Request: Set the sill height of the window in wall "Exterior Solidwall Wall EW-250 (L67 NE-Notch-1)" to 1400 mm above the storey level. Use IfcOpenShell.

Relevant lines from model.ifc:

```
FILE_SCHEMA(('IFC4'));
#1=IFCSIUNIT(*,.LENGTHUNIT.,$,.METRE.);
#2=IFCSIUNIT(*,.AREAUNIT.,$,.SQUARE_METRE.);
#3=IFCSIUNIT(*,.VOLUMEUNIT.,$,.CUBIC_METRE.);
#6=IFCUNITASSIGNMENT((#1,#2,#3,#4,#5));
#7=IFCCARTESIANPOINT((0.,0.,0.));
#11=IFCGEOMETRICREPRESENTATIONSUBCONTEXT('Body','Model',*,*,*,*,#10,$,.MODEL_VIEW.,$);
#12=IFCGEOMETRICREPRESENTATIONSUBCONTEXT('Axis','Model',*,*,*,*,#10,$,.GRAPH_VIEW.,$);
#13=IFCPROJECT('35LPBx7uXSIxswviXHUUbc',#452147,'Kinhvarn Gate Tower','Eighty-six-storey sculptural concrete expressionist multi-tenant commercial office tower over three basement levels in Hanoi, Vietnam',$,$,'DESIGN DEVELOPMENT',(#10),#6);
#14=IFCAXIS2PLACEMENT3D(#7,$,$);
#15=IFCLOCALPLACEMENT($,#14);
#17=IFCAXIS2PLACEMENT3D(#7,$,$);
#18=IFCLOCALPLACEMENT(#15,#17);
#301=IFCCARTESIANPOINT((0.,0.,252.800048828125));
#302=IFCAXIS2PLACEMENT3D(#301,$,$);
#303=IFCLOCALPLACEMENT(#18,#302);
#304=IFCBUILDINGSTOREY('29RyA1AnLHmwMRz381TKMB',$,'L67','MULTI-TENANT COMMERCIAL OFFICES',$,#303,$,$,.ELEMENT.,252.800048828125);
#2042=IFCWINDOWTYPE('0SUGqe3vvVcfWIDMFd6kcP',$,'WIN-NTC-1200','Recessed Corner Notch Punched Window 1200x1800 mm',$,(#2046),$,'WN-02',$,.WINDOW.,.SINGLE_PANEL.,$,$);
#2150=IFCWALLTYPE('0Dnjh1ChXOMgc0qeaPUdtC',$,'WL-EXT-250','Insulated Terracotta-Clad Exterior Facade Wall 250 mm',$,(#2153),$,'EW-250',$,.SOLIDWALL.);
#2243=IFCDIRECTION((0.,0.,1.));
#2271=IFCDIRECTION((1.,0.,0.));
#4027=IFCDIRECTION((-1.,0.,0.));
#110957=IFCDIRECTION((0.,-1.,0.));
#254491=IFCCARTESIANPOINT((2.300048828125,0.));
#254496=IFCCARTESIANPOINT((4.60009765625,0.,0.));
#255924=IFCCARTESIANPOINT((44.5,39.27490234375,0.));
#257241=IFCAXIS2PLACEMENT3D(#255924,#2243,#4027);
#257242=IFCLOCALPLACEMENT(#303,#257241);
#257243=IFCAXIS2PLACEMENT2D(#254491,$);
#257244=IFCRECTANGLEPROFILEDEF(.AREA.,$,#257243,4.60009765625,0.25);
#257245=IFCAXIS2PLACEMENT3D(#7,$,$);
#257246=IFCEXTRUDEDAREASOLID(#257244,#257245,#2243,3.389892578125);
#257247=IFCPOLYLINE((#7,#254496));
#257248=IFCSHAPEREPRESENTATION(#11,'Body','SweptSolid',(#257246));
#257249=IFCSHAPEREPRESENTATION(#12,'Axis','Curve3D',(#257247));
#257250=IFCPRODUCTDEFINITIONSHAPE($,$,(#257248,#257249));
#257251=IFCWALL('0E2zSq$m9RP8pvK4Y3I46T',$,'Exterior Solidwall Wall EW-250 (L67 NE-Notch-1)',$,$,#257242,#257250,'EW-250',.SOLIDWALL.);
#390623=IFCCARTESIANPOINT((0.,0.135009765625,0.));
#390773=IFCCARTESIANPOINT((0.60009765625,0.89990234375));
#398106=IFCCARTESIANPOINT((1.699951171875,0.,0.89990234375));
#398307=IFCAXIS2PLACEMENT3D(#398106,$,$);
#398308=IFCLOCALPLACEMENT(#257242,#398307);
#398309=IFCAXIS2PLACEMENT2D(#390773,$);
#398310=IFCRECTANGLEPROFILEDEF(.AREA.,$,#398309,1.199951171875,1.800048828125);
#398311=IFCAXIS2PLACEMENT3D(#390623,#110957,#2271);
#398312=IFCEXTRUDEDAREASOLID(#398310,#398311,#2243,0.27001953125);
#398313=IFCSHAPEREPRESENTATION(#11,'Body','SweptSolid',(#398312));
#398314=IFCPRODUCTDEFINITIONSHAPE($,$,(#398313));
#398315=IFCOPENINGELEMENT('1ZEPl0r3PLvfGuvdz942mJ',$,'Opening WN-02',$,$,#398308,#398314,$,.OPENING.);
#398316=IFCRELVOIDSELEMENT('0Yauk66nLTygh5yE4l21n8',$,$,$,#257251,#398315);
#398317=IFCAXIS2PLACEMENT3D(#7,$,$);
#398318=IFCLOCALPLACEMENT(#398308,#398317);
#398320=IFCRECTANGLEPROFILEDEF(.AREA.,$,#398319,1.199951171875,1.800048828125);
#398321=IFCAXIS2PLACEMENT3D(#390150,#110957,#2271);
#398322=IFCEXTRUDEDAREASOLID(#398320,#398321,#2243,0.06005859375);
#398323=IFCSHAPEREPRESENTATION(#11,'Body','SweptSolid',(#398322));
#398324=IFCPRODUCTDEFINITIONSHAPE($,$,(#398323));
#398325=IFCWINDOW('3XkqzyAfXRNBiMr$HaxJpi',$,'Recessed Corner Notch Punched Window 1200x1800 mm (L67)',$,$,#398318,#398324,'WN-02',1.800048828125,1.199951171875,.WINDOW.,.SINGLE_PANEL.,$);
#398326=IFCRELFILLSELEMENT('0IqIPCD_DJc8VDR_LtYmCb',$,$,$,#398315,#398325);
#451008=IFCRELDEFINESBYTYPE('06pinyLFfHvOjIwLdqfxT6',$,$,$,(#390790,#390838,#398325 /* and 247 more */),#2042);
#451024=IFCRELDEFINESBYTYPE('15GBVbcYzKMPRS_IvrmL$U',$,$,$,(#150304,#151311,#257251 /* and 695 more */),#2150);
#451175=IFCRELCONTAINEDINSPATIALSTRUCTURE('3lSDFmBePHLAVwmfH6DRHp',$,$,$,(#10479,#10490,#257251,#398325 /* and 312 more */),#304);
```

```python
import numpy as np
import ifcopenshell
import ifcopenshell.api.geometry
import ifcopenshell.geom
import ifcopenshell.util.element
import ifcopenshell.util.placement
import ifcopenshell.util.shape
import ifcopenshell.util.unit

model = ifcopenshell.open("model.ifc")
unit_scale = ifcopenshell.util.unit.calculate_unit_scale(model)

window = model.by_guid("3XkqzyAfXRNBiMr$HaxJpi")
opening = window.FillsVoids[0].RelatingOpeningElement
storey = ifcopenshell.util.element.get_container(window, ifc_class="IfcBuildingStorey")
level = ifcopenshell.util.placement.get_local_placement(storey.ObjectPlacement)[2, 3]

# The opening's origin need not be at the sill, so measure its lowest point.
shape = ifcopenshell.geom.create_shape(ifcopenshell.geom.settings(), opening)
bottom = ifcopenshell.util.shape.get_shape_bottom_elevation(shape, shape.geometry) / unit_scale
dz = level + 1.4 - bottom

shift = np.array([0.0, 0.0, dz])
# The window is placed relative to its opening, so it follows when the opening moves.
matrix = ifcopenshell.util.placement.get_local_placement(opening.ObjectPlacement)
matrix[:3, 3] += shift
ifcopenshell.api.geometry.edit_object_placement(
    model, product=opening, matrix=matrix, is_si=False, should_transform_children=True
)

print(f"moved by {dz * unit_scale:+.3f} m")

model.write("model_v2.ifc")
```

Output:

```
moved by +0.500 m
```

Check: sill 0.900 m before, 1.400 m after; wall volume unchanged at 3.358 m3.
